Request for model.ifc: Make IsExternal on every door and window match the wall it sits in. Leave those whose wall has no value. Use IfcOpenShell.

First a look at what the model holds.

```python
import ifcopenshell
import ifcopenshell.util.element

model = ifcopenshell.open("model.ifc")
print(model.schema)
seen = {}
for e in model.by_type("IfcDoor") + model.by_type("IfcWindow"):
    if not e.FillsVoids:
        continue
    host = e.FillsVoids[0].RelatingOpeningElement.VoidsElements[0].RelatingBuildingElement
    own = ifcopenshell.util.element.get_pset(e, f"Pset_{e.is_a()[3:].removesuffix('StandardCase')}Common", "IsExternal")
    wall = ifcopenshell.util.element.get_pset(host, "Pset_WallCommon", "IsExternal")
    seen[e.is_a(), own, wall] = seen.get((e.is_a(), own, wall), 0) + 1
for (cls, own, wall), count in sorted(seen.items(), key=str):
    print(count, cls, "IsExternal:", own, "| host wall:", wall)
```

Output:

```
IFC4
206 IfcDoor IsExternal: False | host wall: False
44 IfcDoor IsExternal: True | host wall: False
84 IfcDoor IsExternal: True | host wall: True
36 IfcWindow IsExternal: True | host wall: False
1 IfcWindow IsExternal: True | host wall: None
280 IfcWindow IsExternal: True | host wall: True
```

```python
import ifcopenshell
import ifcopenshell.api.pset
import ifcopenshell.util.element

model = ifcopenshell.open("model.ifc")

count = 0
for ifc_class, pset_name in (("IfcDoor", "Pset_DoorCommon"), ("IfcWindow", "Pset_WindowCommon")):
    for e in model.by_type(ifc_class):
        if not e.FillsVoids:
            continue
        host = e.FillsVoids[0].RelatingOpeningElement.VoidsElements[0].RelatingBuildingElement
        external = ifcopenshell.util.element.get_pset(host, "Pset_WallCommon", "IsExternal")
        if external is None or ifcopenshell.util.element.get_pset(e, pset_name, "IsExternal") == external:
            continue
        pset = ifcopenshell.api.pset.add_pset(model, product=e, name=pset_name)
        ifcopenshell.api.pset.edit_pset(model, pset=pset, properties={"IsExternal": external})
        count += 1

print(count, "updated")

model.write("model_edited.ifc")
```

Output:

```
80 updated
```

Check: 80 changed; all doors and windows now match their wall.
